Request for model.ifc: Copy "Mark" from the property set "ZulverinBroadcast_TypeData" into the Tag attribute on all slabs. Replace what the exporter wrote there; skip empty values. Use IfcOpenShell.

First a look at what the model holds.

```python
import ifcopenshell
import ifcopenshell.util.element

model = ifcopenshell.open("model.ifc")
print(model.schema)
slabs = model.by_type("IfcSlab")
print(len(slabs), "slabs")
for e in slabs[:8]:
    source = ifcopenshell.util.element.get_pset(e, "ZulverinBroadcast_TypeData", "Mark")
    target = e.Tag
    print(e.id(), repr(source), repr(target), sep=" | ")
```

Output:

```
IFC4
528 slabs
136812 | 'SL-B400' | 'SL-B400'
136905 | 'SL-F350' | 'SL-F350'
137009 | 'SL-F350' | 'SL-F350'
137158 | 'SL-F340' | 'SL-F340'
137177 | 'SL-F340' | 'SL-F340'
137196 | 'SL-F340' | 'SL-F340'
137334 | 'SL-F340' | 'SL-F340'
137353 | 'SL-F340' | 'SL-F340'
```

```python
import ifcopenshell
import ifcopenshell.util.element

model = ifcopenshell.open("model.ifc")

count = 0
for e in model.by_type("IfcSlab"):
    value = ifcopenshell.util.element.get_pset(e, "ZulverinBroadcast_TypeData", "Mark")
    current = e.Tag
    if not value or not value.strip() or current == value:
        continue
    e.Tag = value
    count += 1

print(count, "slabs updated")

model.write("model_edited.ifc")
```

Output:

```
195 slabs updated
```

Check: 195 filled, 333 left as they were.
